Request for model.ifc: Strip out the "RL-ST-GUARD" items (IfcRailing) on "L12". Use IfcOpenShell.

First a look at what the model holds.

```python
import ifcopenshell
import ifcopenshell.util.element

model = ifcopenshell.open("model.ifc")
print(model.schema)
storey = next(s for s in model.by_type("IfcBuildingStorey") if s.Name == "L12")
railings = [e for e in ifcopenshell.util.element.get_decomposition(storey) if e.is_a("IfcRailing")]
seen = {}
for e in railings:
    element_type = ifcopenshell.util.element.get_type(e)
    name = element_type.Name if element_type not in (None, e) else None
    seen[name] = seen.get(name, 0) + 1
for name, count in sorted(seen.items(), key=str):
    print(count, "x", name)
```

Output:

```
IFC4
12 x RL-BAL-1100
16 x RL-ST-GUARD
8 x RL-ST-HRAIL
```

```python
import ifcopenshell
import ifcopenshell.api.root
import ifcopenshell.util.element

model = ifcopenshell.open("model.ifc")

storey = next(s for s in model.by_type("IfcBuildingStorey") if s.Name == "L12")
railings = [e for e in ifcopenshell.util.element.get_decomposition(storey) if e.is_a("IfcRailing")]
targets = [e for e in railings if (t := ifcopenshell.util.element.get_type(e)) not in (None, e) and t.Name == "RL-ST-GUARD"]

for e in targets:
    ifcopenshell.api.root.remove_product(model, product=e)
print(len(targets), "removed")

model.write("model_edited.ifc")
```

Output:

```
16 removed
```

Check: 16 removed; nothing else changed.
